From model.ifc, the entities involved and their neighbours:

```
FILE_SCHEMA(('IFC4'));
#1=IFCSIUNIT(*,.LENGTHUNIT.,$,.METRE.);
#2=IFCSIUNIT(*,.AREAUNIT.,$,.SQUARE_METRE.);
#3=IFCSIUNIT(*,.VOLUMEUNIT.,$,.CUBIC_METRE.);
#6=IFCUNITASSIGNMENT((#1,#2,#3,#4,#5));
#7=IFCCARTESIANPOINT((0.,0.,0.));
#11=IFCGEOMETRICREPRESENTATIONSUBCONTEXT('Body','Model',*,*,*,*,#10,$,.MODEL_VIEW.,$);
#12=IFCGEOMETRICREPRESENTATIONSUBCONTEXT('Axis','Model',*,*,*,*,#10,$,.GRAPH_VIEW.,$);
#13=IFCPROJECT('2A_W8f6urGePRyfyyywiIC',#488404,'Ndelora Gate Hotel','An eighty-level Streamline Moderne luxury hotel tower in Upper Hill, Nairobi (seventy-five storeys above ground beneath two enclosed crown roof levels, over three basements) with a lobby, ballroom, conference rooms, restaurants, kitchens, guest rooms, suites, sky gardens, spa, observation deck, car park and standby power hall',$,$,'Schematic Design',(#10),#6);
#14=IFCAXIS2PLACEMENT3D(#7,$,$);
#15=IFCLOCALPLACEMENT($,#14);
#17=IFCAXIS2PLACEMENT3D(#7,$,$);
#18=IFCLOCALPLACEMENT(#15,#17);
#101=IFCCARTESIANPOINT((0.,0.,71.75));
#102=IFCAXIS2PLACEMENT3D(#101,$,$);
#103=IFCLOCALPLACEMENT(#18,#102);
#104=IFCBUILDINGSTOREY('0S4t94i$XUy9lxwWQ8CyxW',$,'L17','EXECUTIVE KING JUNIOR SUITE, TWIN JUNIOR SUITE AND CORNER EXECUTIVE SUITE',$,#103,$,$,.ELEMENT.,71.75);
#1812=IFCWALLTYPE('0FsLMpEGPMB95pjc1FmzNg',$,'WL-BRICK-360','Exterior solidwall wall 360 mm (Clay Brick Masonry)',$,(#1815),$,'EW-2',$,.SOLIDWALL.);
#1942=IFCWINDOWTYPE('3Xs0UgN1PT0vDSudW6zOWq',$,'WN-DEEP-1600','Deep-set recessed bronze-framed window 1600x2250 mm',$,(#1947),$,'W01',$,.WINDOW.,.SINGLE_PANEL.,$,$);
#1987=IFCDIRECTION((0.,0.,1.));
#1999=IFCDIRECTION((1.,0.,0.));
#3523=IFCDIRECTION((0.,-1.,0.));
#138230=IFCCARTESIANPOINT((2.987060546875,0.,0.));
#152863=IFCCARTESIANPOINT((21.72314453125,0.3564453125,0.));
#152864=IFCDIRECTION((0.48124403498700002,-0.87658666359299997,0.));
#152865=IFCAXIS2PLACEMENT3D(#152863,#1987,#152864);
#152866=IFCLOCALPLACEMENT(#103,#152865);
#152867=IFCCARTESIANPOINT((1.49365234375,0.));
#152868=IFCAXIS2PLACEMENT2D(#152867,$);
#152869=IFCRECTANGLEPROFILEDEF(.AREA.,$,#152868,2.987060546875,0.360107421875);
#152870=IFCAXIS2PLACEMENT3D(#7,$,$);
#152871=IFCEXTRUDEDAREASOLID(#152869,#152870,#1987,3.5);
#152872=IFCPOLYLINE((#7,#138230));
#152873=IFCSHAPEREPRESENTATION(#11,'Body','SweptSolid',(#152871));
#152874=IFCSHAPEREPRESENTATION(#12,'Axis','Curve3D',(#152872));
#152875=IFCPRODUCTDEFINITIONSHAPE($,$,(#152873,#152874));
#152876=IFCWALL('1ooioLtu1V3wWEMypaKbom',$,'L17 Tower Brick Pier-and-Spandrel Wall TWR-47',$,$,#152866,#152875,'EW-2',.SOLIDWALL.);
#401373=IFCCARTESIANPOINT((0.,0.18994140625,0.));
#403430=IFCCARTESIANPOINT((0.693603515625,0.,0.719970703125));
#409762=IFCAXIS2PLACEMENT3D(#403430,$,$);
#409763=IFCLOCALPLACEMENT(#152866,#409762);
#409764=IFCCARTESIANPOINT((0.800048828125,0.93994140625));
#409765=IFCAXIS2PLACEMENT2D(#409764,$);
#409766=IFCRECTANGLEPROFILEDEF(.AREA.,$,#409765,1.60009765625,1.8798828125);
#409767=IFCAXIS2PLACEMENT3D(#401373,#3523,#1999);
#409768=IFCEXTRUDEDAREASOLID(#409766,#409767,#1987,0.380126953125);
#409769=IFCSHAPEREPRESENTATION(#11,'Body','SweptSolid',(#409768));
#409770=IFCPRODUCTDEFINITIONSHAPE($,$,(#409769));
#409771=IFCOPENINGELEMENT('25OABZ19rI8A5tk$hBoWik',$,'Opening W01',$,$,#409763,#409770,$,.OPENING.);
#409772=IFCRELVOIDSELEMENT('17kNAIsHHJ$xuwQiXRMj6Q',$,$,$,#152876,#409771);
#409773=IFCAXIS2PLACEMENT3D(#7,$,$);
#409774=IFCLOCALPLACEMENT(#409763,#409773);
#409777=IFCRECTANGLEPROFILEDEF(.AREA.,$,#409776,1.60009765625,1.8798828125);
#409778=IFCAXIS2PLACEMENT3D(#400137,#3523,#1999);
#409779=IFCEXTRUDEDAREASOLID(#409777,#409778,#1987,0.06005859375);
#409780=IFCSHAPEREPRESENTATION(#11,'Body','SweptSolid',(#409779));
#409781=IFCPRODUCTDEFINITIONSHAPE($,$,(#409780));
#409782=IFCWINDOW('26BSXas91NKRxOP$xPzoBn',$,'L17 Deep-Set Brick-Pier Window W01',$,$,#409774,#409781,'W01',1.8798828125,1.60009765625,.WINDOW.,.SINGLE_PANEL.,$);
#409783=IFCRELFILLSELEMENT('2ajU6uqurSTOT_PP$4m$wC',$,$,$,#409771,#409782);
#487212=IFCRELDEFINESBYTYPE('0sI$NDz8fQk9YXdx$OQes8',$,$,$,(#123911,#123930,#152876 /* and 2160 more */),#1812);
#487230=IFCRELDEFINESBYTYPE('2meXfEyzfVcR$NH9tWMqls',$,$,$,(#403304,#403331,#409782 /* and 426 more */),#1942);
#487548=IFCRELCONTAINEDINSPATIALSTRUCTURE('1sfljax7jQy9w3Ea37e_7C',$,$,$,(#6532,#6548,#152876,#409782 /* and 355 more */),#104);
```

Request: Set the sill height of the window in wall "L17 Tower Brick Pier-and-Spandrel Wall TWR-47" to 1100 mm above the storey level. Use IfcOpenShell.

```python
import numpy as np
import ifcopenshell
import ifcopenshell.api.geometry
import ifcopenshell.geom
import ifcopenshell.util.element
import ifcopenshell.util.placement
import ifcopenshell.util.shape
import ifcopenshell.util.unit

model = ifcopenshell.open("model.ifc")
unit_scale = ifcopenshell.util.unit.calculate_unit_scale(model)

window = model.by_guid("26BSXas91NKRxOP$xPzoBn")
opening = window.FillsVoids[0].RelatingOpeningElement
storey = ifcopenshell.util.element.get_container(window, ifc_class="IfcBuildingStorey")
level = ifcopenshell.util.placement.get_local_placement(storey.ObjectPlacement)[2, 3]

# The opening's origin need not be at the sill, so measure its lowest point.
shape = ifcopenshell.geom.create_shape(ifcopenshell.geom.settings(), opening)
bottom = ifcopenshell.util.shape.get_shape_bottom_elevation(shape, shape.geometry) / unit_scale
dz = level + 1.1 - bottom

shift = np.array([0.0, 0.0, dz])
# The window is placed relative to its opening, so it follows when the opening moves.
matrix = ifcopenshell.util.placement.get_local_placement(opening.ObjectPlacement)
matrix[:3, 3] += shift
ifcopenshell.api.geometry.edit_object_placement(
    model, product=opening, matrix=matrix, is_si=False, should_transform_children=True
)

print(f"moved by {dz * unit_scale:+.3f} m")

model.write("model_edited.ifc")
```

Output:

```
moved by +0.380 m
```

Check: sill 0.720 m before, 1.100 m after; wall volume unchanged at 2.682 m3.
